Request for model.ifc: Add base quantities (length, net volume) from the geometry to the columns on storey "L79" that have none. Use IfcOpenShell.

First a look at what the model holds.

```python
import ifcopenshell
import ifcopenshell.util.element
import ifcopenshell.util.unit

model = ifcopenshell.open("model.ifc")
print(model.schema)
for unit_type in ("LENGTHUNIT", "AREAUNIT", "VOLUMEUNIT"):
    print(unit_type, ifcopenshell.util.unit.calculate_unit_scale(model, unit_type))
storey = next(s for s in model.by_type("IfcBuildingStorey") if s.Name == "L79")
columns = [e for e in ifcopenshell.util.element.get_decomposition(storey) if e.is_a("IfcColumn")]
for e in sorted(columns, key=lambda e: e.id()):
    print(e.id(), e.is_a(), e.Name, list(ifcopenshell.util.element.get_psets(e, qtos_only=True)), sep=" | ")
```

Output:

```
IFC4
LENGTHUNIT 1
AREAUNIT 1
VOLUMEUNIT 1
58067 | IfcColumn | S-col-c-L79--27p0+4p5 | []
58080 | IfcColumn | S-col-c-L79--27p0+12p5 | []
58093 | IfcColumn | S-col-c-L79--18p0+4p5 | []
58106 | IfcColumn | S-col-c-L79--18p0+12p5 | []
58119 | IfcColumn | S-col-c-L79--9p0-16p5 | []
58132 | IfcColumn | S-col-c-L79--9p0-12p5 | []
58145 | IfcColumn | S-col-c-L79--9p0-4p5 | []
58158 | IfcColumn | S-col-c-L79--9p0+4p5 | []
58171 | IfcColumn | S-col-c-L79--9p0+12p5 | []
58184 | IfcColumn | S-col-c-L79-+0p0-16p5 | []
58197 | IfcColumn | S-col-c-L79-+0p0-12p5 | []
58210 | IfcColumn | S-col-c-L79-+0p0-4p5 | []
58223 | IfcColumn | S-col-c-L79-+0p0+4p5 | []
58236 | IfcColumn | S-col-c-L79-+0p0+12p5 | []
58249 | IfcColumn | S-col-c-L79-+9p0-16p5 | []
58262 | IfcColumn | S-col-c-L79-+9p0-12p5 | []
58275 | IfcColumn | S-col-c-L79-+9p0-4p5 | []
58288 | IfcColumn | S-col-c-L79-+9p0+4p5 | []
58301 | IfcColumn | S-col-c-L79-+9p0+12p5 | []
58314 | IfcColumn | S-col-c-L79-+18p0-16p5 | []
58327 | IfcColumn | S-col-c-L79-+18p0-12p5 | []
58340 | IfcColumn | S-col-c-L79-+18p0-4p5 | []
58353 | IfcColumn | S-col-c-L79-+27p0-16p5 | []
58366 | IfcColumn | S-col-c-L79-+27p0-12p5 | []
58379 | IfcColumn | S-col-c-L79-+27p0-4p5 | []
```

```python
import ifcopenshell
import ifcopenshell.api.pset
import ifcopenshell.geom
import ifcopenshell.util.element
import ifcopenshell.util.shape
import ifcopenshell.util.unit

model = ifcopenshell.open("model.ifc")
unit_scale = ifcopenshell.util.unit.calculate_unit_scale(model)
volume_scale = ifcopenshell.util.unit.calculate_unit_scale(model, "VOLUMEUNIT")
settings = ifcopenshell.geom.settings()

storey = next(s for s in model.by_type("IfcBuildingStorey") if s.Name == "L79")
columns = [e for e in ifcopenshell.util.element.get_decomposition(storey) if e.is_a("IfcColumn")]

for e in sorted(columns, key=lambda e: e.id()):
    if ifcopenshell.util.element.get_psets(e, qtos_only=True, should_inherit=False):
        continue
    # Geometry comes back in metres, in the element's own axes.
    shape = ifcopenshell.geom.create_shape(settings, e)
    values = {
        "Length": ifcopenshell.util.shape.get_z(shape.geometry) / unit_scale,
        "NetVolume": ifcopenshell.util.shape.get_volume(shape.geometry) / volume_scale,
    }
    qto = ifcopenshell.api.pset.add_qto(model, product=e, name="Qto_ColumnBaseQuantities")
    ifcopenshell.api.pset.edit_qto(model, qto=qto, properties=values)
    print(e.id(), {k: round(v, 3) for k, v in values.items()})

model.write("model-out.ifc")
```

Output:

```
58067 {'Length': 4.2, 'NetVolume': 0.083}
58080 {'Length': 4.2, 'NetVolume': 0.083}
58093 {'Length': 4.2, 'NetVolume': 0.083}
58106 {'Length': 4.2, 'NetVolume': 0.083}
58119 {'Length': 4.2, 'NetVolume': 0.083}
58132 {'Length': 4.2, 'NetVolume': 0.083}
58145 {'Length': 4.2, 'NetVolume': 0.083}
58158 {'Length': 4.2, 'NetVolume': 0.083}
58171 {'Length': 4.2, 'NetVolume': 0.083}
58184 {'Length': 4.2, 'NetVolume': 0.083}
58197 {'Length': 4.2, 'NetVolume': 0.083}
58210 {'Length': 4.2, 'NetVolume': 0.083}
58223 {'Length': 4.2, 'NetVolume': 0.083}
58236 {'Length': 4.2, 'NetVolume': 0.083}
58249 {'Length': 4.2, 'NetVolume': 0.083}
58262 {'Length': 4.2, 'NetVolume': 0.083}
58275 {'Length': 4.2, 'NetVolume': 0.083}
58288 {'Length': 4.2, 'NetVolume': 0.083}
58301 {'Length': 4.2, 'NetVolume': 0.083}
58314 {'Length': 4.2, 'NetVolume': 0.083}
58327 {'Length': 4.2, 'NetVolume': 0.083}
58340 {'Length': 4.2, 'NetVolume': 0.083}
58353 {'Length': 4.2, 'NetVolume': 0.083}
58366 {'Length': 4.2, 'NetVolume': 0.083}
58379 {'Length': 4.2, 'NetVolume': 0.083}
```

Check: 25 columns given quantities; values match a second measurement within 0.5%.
